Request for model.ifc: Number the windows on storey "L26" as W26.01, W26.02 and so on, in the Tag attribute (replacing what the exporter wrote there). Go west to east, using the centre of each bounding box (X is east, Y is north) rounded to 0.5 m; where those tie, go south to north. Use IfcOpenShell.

First a look at what the model holds.

```python
import ifcopenshell
import ifcopenshell.util.element
import ifcopenshell.util.placement

model = ifcopenshell.open("model.ifc")
print(model.schema)
storey = next(s for s in model.by_type("IfcBuildingStorey") if s.Name == "L26")
windows = [e for e in ifcopenshell.util.element.get_decomposition(storey) if e.is_a("IfcWindow")]
for e in sorted(windows, key=lambda e: e.id()):
    origin = ifcopenshell.util.placement.get_local_placement(e.ObjectPlacement)[:3, 3]
    print(e.id(), e.Tag, e.Name, origin.round(2) + 0.0, sep=" | ")
```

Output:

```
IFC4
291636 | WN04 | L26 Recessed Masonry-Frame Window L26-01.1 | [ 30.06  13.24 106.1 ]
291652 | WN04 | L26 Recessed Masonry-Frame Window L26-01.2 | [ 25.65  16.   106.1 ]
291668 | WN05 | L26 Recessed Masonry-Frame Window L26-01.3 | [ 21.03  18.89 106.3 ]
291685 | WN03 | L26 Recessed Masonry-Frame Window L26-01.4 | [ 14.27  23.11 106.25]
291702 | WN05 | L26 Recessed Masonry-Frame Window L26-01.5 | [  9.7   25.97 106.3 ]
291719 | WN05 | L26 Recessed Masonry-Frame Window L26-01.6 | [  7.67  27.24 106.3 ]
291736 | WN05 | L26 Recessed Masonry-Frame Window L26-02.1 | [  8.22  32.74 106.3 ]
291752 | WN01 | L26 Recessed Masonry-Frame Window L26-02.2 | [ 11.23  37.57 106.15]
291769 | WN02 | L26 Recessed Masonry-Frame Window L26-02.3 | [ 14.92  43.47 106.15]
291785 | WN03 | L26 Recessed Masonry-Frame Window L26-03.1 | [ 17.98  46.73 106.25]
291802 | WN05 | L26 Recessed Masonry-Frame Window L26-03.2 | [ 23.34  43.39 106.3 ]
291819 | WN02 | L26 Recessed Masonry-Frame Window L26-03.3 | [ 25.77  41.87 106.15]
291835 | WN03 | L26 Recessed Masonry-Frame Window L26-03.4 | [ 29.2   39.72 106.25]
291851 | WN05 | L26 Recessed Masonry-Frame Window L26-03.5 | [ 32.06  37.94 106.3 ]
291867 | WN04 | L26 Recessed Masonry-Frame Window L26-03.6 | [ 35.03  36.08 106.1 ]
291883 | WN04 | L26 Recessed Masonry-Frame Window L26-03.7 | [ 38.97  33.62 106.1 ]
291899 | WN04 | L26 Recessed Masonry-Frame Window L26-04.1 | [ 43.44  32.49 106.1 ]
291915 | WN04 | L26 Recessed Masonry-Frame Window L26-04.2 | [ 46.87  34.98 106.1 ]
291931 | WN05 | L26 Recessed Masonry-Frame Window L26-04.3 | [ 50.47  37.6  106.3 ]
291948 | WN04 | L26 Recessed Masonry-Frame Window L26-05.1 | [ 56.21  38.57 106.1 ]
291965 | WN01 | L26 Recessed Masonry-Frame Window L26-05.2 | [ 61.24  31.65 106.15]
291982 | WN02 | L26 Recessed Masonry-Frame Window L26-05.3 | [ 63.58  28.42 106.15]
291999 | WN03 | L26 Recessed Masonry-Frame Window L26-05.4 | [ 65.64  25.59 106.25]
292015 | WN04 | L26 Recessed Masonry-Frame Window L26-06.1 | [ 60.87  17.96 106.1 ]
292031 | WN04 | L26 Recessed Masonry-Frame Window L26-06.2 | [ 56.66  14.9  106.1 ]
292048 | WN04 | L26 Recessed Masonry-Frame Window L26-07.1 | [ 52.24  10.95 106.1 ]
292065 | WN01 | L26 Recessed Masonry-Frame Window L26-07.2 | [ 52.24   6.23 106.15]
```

```python
import ifcopenshell
import ifcopenshell.geom
import ifcopenshell.util.element
import ifcopenshell.util.shape

model = ifcopenshell.open("model.ifc")
settings = ifcopenshell.geom.settings()
settings.set("use-world-coords", True)


def centre(element):
    shape = ifcopenshell.geom.create_shape(settings, element)
    return ifcopenshell.util.shape.get_bbox_centroid(shape.geometry)


storey = next(s for s in model.by_type("IfcBuildingStorey") if s.Name == "L26")
windows = [e for e in ifcopenshell.util.element.get_decomposition(storey) if e.is_a("IfcWindow")]

# Insertion points can sit at a corner or the storey origin, so sort by the geometry (in metres).
centres = {e: centre(e) for e in windows}
windows.sort(key=lambda e: (round(centres[e][0] / 0.5), centres[e][1]))

for i, e in enumerate(windows, start=1):
    number = f"W26.{i:02d}"
    e.Tag = number
    print(e.id(), number)

model.write("model_rev.ifc")
```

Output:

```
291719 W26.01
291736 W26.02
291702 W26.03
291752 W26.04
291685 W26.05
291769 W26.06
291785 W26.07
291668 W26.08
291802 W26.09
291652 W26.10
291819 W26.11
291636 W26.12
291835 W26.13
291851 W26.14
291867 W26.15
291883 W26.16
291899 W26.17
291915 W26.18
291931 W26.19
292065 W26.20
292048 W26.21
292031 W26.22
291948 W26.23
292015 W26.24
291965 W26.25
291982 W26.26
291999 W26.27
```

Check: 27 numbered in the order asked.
